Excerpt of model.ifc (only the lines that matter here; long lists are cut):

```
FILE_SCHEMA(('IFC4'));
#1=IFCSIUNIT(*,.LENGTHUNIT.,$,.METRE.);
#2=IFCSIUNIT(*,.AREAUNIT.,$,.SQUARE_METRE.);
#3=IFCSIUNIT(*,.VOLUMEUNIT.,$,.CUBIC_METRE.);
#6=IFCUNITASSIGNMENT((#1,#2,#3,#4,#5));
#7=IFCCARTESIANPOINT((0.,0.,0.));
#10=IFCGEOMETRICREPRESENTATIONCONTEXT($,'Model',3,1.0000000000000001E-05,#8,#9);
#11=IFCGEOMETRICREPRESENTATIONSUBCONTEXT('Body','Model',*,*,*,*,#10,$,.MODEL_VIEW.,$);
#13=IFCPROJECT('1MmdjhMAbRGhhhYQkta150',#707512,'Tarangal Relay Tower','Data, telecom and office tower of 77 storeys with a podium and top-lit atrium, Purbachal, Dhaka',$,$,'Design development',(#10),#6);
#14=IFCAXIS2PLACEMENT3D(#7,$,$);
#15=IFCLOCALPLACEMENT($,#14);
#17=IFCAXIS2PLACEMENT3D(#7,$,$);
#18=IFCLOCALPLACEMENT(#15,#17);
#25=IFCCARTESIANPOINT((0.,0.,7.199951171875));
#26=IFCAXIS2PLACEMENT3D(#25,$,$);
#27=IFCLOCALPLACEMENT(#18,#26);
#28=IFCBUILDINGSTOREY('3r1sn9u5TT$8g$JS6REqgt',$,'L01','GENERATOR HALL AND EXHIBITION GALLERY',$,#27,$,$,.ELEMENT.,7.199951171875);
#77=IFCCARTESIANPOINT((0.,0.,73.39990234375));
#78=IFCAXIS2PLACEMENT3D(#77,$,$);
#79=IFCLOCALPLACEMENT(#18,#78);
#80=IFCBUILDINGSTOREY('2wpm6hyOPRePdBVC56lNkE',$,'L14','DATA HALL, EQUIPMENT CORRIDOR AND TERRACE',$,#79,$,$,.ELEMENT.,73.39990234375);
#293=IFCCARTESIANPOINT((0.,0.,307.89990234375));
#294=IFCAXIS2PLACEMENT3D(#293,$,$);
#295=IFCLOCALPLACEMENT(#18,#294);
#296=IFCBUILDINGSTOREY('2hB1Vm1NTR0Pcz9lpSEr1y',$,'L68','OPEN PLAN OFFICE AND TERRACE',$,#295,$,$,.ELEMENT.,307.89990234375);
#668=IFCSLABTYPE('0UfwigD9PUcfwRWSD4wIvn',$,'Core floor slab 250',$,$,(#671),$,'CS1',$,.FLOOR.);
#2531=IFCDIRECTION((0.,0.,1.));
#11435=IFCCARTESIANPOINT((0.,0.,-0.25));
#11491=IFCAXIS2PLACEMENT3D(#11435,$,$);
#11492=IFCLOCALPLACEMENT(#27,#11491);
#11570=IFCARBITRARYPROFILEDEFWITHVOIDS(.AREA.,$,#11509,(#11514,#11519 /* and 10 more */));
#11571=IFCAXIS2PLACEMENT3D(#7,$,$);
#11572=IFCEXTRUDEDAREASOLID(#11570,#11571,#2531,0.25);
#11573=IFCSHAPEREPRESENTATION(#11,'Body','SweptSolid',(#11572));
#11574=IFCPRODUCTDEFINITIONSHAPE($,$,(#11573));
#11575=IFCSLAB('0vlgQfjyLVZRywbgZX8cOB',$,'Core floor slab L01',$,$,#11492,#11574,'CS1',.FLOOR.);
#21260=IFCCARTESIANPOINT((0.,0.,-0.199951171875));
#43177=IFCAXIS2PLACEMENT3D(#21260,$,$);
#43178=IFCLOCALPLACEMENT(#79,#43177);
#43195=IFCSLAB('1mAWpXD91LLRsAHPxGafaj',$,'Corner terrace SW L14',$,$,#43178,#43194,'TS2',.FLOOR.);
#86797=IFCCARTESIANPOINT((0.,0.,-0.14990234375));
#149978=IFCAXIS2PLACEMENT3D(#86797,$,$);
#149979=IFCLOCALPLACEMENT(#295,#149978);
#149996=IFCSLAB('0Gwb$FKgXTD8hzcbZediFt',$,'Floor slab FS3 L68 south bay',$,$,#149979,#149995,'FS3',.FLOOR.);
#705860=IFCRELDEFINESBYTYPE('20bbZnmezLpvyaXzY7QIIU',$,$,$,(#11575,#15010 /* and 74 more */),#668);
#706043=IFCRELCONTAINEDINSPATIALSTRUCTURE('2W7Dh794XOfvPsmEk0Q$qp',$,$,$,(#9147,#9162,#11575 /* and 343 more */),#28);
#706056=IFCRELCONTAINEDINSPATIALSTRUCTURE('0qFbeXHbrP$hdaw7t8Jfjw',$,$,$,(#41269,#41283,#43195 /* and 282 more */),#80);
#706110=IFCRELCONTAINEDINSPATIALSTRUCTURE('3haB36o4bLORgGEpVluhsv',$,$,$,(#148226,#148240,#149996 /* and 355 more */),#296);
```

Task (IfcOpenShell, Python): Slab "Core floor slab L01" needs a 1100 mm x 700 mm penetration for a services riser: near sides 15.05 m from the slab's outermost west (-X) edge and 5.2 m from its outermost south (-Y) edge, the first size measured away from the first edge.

```python
import numpy as np
import ifcopenshell
import ifcopenshell.api.feature
import ifcopenshell.api.geometry
import ifcopenshell.api.root
import ifcopenshell.geom
import ifcopenshell.util.placement
import ifcopenshell.util.representation
import ifcopenshell.util.shape
import ifcopenshell.util.unit

model = ifcopenshell.open("model.ifc")
unit_scale = ifcopenshell.util.unit.calculate_unit_scale(model)
settings = ifcopenshell.geom.settings()


def volume(element):
    """Net volume in cubic metres, openings subtracted."""
    shape = ifcopenshell.geom.create_shape(settings, element)
    return ifcopenshell.util.shape.get_volume(shape.geometry)


slab = model.by_id(11575)
before = volume(slab)

# Extent in the slab's own axes, in metres. The edges named are its -X and -Y sides.
slab_shape = ifcopenshell.geom.create_shape(settings, slab)
vertices = ifcopenshell.util.shape.get_vertices(slab_shape.geometry)
x_min, y_min, bottom = vertices.min(axis=0)
top = vertices[:, 2].max()

opening = ifcopenshell.api.root.create_entity(model, ifc_class="IfcOpeningElement", name="Services riser opening", predefined_type="OPENING")
context = ifcopenshell.util.representation.get_context(model, "Model", "Body", "MODEL_VIEW")
width, depth = 1.1, 0.7
outline = [(0.0, 0.0), (width, 0.0), (width, depth), (0.0, depth), (0.0, 0.0)]
# Overshoot both faces by 50 mm so the cut is clean.
shape = ifcopenshell.api.geometry.add_slab_representation(
    model, context=context, depth=top - bottom + 0.1, polyline=outline
)
ifcopenshell.api.geometry.assign_representation(model, product=opening, representation=shape)

matrix = ifcopenshell.util.placement.get_local_placement(slab.ObjectPlacement)
matrix[:, 3] = matrix @ np.append(np.array([x_min + 15.05, y_min + 5.2, bottom - 0.05]) / unit_scale, 1.0)
ifcopenshell.api.geometry.edit_object_placement(model, product=opening, matrix=matrix, is_si=False)
ifcopenshell.api.feature.add_feature(model, feature=opening, element=slab)

after = volume(slab)

print(f"slab volume {before:.3f} -> {after:.3f} m3")

model.write("model-out.ifc")
```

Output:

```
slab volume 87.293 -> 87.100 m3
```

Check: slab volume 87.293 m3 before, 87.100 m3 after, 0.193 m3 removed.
